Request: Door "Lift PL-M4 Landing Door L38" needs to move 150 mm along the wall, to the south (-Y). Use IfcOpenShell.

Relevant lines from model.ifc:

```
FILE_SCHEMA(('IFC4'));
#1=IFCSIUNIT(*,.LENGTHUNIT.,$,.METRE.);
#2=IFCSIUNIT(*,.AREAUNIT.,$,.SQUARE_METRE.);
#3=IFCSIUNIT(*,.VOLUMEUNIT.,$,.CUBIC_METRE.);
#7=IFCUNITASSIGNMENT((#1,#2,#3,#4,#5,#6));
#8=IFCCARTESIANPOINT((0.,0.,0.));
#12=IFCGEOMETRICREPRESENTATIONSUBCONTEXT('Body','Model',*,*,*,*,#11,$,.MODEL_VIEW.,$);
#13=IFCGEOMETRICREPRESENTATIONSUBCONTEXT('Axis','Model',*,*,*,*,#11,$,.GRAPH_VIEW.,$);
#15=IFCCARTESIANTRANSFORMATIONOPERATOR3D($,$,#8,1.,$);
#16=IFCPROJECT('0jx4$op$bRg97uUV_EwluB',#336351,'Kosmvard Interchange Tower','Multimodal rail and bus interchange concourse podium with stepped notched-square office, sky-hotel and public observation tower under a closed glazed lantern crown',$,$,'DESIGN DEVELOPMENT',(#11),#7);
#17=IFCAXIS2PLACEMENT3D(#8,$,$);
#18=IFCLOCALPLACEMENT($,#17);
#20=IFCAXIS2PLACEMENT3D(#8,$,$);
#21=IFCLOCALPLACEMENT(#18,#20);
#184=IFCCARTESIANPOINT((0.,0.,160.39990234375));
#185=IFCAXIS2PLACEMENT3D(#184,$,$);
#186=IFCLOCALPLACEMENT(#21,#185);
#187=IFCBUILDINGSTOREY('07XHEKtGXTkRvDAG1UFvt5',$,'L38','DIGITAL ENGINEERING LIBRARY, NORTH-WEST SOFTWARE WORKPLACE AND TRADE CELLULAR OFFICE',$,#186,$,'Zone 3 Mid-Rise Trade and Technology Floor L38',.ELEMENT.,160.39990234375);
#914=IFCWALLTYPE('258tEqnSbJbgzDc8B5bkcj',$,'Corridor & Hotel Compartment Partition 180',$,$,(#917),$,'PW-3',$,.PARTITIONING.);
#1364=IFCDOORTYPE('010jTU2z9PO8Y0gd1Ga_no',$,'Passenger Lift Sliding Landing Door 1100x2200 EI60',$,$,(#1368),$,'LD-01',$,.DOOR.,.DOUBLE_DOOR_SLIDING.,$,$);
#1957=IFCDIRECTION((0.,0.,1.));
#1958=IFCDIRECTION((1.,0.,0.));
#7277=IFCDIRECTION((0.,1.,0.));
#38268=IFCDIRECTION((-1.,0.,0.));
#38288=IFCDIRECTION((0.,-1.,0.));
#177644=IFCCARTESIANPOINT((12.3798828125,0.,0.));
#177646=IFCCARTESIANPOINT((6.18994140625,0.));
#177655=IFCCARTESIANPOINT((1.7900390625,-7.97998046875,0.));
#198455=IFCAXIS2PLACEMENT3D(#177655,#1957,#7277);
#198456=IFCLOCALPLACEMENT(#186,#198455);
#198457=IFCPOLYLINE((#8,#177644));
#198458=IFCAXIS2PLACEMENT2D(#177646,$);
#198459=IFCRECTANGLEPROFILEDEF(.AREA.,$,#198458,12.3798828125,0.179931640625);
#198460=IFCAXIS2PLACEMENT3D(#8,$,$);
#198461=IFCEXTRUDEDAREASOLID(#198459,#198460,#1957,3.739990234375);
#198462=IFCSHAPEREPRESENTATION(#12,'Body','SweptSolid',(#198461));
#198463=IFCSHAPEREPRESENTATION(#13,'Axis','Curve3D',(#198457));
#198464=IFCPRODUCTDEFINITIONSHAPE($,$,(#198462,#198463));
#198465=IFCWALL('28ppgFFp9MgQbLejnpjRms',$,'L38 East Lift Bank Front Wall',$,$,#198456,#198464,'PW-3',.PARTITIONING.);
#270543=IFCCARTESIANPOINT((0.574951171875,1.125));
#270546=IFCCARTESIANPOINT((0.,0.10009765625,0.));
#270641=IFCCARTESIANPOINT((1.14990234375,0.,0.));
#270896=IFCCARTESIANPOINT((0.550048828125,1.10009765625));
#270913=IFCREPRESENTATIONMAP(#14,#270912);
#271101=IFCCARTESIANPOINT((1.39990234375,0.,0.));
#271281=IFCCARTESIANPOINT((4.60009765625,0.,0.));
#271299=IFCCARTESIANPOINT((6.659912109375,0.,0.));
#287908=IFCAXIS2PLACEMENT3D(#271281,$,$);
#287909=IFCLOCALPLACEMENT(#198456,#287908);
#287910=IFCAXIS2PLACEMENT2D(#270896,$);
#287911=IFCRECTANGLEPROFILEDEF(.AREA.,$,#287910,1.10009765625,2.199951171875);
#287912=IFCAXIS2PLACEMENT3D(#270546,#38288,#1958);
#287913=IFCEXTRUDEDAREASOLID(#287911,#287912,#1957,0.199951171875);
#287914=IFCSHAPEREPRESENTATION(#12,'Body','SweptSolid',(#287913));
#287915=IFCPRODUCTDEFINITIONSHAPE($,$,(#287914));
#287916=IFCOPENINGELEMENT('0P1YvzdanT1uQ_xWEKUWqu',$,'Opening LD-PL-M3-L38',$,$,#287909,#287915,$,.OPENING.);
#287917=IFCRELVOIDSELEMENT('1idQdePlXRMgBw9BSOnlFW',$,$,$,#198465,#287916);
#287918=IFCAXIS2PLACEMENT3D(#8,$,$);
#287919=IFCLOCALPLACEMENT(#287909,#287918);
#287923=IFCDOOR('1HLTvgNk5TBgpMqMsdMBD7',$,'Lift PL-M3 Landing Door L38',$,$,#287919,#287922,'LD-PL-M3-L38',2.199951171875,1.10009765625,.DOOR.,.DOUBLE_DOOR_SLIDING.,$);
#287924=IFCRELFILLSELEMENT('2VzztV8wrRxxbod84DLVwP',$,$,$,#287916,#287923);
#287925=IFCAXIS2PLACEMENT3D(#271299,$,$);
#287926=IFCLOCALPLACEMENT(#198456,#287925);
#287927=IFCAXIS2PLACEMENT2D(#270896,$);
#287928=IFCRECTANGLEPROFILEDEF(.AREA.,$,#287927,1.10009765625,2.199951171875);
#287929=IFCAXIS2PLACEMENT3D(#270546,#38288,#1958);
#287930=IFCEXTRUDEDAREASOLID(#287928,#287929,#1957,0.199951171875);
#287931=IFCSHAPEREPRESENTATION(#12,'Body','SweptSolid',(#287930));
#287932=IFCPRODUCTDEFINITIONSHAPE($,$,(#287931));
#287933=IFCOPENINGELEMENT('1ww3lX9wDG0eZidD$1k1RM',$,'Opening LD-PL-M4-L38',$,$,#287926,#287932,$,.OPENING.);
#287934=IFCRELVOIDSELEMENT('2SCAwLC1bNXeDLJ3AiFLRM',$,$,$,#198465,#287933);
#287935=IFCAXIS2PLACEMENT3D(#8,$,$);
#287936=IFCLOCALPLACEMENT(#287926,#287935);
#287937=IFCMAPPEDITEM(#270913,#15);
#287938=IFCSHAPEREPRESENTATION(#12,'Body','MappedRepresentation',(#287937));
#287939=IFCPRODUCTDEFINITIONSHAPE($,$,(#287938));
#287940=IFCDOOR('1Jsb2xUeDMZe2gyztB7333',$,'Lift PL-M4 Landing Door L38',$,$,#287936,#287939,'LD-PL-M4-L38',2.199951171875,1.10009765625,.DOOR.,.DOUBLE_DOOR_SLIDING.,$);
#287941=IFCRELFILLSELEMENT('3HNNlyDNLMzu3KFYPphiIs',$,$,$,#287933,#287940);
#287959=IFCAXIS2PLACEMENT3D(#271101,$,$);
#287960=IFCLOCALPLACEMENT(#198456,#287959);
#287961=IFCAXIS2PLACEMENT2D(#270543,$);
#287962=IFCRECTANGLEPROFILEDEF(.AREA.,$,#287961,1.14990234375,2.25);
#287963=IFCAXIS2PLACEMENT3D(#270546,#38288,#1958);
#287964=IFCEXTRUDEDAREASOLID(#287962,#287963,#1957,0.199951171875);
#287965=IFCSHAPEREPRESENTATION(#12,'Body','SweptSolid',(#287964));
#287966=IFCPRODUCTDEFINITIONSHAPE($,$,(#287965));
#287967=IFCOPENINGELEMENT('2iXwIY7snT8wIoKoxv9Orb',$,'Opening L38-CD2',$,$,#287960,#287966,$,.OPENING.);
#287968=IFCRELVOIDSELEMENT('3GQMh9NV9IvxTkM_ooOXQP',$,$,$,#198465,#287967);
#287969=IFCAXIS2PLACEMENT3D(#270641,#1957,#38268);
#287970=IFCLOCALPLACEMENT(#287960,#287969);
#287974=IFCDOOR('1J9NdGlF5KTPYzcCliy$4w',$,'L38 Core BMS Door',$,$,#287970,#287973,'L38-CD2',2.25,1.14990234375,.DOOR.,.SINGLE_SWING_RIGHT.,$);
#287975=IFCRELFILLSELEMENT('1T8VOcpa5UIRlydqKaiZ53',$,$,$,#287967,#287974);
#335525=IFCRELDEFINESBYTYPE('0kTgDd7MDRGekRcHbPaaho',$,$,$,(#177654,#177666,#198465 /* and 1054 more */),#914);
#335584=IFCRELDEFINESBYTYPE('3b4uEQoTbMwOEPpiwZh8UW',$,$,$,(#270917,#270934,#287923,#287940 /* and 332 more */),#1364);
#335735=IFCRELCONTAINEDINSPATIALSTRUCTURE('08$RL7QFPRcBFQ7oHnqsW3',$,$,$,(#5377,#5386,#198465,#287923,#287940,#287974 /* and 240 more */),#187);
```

```python
import ifcopenshell
import ifcopenshell.api.geometry
import ifcopenshell.util.placement

model = ifcopenshell.open("model.ifc")

door = model.by_guid("1Jsb2xUeDMZe2gyztB7333")
opening = door.FillsVoids[0].RelatingOpeningElement
wall = opening.VoidsElements[0].RelatingBuildingElement

wall_matrix = ifcopenshell.util.placement.get_local_placement(wall.ObjectPlacement)
shift = wall_matrix[:3, 0] * -0.15
before = ifcopenshell.util.placement.get_local_placement(door.ObjectPlacement)[:3, 3].copy()

# The door is placed relative to its opening, so it follows when the opening moves.
matrix = ifcopenshell.util.placement.get_local_placement(opening.ObjectPlacement)
matrix[:3, 3] += shift
ifcopenshell.api.geometry.edit_object_placement(
    model, product=opening, matrix=matrix, is_si=False, should_transform_children=True
)

after = ifcopenshell.util.placement.get_local_placement(door.ObjectPlacement)[:3, 3]
print("door moved by", (after - before).round(3) + 0.0)

model.write("model_rev.ifc")
```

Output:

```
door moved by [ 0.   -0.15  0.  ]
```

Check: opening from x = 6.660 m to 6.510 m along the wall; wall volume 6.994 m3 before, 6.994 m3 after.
